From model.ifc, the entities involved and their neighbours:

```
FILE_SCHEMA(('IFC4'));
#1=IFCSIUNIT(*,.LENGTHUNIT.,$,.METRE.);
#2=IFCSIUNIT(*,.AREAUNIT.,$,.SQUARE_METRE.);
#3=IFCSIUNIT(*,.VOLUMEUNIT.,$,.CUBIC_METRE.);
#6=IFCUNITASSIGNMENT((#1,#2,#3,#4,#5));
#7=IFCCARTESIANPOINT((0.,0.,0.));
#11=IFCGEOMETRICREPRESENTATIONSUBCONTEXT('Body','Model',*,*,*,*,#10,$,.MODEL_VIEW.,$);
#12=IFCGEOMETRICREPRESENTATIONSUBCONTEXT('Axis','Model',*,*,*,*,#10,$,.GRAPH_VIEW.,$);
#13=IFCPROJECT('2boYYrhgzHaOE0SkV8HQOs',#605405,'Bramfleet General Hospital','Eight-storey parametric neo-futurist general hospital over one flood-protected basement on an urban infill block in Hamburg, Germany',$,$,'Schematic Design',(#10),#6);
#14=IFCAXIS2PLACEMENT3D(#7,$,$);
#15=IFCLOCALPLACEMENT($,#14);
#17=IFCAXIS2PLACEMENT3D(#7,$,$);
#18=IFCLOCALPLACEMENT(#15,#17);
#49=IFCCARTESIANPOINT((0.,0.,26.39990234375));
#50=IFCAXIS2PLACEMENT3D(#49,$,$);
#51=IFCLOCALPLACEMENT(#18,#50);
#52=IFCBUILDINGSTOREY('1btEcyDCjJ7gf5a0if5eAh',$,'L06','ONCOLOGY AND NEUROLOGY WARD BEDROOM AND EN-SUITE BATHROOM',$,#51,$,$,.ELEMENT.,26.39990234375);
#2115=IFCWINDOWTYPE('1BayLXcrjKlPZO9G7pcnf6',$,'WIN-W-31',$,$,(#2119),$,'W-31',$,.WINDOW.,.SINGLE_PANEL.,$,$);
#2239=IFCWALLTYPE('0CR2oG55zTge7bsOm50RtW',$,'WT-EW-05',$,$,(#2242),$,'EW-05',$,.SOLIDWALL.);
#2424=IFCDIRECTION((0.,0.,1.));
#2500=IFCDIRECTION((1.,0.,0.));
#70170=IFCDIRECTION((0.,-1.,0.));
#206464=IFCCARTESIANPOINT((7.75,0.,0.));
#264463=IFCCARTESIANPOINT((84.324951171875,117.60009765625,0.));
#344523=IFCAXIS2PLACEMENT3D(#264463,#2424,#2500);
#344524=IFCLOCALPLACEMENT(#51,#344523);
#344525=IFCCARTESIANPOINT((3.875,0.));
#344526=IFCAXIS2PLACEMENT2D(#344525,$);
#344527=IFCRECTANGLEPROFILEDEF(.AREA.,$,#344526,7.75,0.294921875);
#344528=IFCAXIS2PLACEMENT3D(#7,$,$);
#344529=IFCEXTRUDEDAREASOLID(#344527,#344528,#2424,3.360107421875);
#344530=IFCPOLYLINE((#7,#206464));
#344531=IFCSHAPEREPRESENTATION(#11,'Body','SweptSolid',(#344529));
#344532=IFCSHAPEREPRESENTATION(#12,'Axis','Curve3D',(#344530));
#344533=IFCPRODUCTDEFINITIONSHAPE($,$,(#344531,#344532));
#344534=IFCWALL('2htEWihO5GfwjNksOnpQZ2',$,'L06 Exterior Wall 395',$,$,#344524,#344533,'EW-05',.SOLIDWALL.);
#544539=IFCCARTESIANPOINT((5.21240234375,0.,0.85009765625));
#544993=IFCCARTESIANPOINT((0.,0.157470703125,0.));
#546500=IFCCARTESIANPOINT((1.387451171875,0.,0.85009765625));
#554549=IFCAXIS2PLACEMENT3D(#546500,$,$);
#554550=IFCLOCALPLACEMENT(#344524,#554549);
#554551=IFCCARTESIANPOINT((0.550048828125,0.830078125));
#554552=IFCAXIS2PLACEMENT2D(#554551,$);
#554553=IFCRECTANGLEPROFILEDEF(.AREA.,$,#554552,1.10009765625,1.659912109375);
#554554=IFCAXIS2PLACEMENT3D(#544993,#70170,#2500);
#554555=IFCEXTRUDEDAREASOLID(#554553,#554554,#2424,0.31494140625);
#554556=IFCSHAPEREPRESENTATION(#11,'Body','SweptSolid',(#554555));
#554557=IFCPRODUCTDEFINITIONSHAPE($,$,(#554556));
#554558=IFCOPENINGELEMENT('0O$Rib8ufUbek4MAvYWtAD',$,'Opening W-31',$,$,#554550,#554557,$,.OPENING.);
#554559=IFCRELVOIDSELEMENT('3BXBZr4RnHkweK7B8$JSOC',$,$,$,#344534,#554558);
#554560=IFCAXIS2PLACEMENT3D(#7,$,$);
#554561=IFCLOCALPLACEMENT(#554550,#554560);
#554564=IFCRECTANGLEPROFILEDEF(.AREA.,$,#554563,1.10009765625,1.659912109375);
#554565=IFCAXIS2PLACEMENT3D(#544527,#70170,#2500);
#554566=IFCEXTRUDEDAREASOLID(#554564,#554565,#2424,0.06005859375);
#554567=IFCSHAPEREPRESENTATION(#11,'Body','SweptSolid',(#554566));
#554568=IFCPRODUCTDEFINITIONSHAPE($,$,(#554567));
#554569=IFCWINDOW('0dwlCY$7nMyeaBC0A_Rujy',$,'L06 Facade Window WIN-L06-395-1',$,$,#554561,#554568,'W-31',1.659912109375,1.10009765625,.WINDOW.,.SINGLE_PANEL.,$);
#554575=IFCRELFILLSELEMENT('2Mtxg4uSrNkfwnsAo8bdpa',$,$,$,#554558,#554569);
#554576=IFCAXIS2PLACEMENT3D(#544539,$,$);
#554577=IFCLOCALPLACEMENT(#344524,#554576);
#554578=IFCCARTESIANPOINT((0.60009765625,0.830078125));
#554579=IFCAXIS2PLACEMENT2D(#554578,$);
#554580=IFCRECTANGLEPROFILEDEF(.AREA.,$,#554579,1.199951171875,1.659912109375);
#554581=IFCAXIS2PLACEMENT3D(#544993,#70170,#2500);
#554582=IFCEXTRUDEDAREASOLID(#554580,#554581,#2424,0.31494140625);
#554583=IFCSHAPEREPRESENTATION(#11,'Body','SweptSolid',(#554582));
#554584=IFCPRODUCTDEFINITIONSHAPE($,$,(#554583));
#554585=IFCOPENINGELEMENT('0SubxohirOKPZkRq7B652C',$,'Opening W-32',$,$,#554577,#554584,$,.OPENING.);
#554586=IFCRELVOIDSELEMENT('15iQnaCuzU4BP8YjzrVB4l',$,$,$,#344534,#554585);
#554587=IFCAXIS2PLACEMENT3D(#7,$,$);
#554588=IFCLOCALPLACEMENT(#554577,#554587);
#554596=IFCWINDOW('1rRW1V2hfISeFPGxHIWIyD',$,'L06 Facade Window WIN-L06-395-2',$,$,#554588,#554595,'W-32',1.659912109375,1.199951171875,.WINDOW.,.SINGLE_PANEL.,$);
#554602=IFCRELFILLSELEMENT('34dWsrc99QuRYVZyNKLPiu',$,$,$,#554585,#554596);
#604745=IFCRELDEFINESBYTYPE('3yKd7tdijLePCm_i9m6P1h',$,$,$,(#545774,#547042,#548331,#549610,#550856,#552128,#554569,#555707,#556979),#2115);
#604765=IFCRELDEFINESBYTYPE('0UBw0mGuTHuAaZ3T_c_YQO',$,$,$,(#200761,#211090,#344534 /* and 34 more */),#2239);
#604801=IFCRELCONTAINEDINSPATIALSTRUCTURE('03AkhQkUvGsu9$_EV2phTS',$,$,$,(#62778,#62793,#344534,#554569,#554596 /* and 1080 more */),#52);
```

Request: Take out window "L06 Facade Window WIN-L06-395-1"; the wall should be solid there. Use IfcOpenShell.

```python
import ifcopenshell
import ifcopenshell.api.feature
import ifcopenshell.api.root
import ifcopenshell.geom
import ifcopenshell.util.shape

model = ifcopenshell.open("model.ifc")
settings = ifcopenshell.geom.settings()


def volume(element):
    """Net volume in cubic metres, openings subtracted."""
    shape = ifcopenshell.geom.create_shape(settings, element)
    return ifcopenshell.util.shape.get_volume(shape.geometry)


window = model.by_id(554569)
opening = window.FillsVoids[0].RelatingOpeningElement
wall = opening.VoidsElements[0].RelatingBuildingElement
before = volume(wall)

ifcopenshell.api.root.remove_product(model, product=window)
ifcopenshell.api.feature.remove_feature(model, feature=opening)

after = volume(wall)

print(f"wall volume {before:.3f} -> {after:.3f} m3")

model.write("model-out.ifc")
```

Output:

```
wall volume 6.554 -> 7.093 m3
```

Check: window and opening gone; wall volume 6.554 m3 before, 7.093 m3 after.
